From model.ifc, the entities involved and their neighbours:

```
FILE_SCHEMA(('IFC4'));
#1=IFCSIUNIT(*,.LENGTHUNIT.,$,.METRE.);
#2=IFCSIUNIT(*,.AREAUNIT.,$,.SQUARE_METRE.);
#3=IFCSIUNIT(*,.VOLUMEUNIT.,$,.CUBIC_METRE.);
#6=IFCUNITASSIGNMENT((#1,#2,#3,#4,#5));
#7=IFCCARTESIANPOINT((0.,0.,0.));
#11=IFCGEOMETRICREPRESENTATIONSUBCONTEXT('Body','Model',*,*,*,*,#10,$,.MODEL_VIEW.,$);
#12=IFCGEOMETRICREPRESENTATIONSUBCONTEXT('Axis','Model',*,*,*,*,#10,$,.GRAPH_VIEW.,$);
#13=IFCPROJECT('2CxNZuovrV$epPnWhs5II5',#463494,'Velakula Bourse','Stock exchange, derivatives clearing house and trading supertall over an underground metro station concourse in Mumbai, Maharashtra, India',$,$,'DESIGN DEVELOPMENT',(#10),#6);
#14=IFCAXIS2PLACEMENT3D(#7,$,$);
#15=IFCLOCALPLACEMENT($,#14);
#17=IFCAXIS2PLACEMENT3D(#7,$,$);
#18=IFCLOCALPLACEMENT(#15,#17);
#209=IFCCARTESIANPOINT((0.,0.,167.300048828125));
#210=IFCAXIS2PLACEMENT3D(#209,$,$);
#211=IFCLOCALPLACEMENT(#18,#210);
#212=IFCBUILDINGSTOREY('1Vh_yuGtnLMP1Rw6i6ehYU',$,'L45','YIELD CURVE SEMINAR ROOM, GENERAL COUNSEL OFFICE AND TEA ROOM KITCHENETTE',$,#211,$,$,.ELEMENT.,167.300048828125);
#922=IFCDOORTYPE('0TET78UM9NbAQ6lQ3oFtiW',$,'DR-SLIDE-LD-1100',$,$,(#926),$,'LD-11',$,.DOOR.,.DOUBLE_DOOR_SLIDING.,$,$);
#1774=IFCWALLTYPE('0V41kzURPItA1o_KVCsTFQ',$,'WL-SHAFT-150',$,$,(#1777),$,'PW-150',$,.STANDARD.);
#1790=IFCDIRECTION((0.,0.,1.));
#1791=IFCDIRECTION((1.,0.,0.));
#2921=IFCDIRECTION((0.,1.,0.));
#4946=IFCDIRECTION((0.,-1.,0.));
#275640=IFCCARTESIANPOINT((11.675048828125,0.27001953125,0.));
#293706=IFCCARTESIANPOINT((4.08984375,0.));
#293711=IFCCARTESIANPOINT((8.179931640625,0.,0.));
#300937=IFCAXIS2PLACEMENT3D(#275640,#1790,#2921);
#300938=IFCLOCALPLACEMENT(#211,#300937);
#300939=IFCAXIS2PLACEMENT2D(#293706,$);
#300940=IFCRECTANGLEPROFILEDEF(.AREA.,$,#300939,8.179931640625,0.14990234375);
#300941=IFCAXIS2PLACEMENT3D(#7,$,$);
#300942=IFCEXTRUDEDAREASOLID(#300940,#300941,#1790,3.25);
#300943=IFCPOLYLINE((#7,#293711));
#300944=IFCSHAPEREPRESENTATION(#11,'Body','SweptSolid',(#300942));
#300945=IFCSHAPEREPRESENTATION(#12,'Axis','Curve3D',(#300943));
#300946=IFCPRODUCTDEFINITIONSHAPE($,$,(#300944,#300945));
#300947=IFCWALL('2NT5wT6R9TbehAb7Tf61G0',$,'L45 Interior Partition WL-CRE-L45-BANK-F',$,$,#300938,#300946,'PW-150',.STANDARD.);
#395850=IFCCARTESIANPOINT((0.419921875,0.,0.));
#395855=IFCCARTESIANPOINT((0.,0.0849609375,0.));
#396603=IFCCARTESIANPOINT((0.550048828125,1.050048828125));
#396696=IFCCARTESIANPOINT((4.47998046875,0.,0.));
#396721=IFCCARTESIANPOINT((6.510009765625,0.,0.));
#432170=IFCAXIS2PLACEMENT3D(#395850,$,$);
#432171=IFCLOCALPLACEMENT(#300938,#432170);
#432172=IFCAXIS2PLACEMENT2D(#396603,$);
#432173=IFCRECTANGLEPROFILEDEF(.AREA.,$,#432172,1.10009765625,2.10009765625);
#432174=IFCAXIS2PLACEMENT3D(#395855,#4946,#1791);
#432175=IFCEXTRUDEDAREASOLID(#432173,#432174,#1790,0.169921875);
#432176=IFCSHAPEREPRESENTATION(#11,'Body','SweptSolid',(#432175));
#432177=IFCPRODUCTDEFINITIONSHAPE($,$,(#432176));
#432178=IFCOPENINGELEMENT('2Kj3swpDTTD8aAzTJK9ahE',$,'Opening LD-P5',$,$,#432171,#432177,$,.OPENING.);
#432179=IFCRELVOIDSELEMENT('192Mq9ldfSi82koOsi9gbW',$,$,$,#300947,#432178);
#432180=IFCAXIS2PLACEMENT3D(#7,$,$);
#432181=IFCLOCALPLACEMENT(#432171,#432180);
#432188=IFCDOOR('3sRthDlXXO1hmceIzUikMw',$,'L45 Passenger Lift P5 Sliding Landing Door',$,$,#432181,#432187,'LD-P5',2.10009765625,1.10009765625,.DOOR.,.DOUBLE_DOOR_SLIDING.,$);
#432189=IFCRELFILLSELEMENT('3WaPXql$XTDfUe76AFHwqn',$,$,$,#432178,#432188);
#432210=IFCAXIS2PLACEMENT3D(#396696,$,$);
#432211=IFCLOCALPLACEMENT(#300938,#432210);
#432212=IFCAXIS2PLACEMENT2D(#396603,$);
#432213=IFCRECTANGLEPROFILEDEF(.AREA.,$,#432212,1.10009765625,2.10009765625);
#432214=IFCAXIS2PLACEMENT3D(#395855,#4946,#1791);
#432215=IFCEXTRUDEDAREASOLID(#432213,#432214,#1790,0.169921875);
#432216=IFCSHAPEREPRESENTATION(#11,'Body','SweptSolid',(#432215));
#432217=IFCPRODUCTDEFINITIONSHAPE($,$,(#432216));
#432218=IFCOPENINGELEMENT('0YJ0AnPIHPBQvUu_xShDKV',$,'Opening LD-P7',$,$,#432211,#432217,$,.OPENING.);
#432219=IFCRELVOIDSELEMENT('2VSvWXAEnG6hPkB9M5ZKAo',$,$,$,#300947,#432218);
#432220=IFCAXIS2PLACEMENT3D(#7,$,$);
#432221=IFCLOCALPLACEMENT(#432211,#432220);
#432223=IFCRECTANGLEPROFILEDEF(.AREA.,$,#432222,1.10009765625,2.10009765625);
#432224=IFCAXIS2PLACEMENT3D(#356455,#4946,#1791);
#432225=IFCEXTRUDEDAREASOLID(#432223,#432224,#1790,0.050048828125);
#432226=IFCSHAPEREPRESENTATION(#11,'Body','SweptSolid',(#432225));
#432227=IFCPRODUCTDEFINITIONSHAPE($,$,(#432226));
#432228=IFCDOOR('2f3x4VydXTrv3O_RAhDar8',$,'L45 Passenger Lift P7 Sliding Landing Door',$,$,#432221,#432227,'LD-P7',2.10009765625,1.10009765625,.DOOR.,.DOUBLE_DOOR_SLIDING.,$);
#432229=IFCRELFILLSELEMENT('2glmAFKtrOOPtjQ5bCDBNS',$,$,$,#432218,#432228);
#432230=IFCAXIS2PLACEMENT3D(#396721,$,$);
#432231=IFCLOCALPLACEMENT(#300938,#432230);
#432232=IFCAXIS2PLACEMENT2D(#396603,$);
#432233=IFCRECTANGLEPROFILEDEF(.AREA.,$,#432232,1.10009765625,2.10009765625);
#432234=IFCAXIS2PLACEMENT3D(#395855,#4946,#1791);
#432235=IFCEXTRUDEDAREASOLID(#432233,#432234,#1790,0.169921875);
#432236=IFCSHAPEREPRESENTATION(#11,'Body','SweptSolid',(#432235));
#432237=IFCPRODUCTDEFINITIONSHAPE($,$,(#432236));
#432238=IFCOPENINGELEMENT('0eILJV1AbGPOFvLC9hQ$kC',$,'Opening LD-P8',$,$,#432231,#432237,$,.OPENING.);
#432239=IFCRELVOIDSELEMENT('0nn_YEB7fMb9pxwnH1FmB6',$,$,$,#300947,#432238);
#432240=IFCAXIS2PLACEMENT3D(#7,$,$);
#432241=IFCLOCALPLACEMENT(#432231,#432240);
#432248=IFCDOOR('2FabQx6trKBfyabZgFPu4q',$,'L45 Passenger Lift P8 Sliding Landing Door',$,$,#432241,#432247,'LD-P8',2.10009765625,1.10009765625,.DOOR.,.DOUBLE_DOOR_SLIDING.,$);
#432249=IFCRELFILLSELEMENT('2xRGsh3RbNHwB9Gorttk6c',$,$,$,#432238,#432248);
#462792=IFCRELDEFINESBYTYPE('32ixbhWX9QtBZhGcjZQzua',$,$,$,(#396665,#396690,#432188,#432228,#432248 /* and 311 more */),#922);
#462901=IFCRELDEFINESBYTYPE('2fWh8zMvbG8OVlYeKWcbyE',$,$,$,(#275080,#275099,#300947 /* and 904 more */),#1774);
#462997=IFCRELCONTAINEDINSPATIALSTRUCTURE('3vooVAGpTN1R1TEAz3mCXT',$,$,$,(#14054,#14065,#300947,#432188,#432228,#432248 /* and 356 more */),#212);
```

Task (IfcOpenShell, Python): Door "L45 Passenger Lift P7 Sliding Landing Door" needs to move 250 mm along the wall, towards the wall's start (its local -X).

```python
import ifcopenshell
import ifcopenshell.api.geometry
import ifcopenshell.util.placement
import ifcopenshell.util.unit

model = ifcopenshell.open("model.ifc")
unit_scale = ifcopenshell.util.unit.calculate_unit_scale(model)

door = model.by_guid("2f3x4VydXTrv3O_RAhDar8")
opening = door.FillsVoids[0].RelatingOpeningElement
wall = opening.VoidsElements[0].RelatingBuildingElement

wall_matrix = ifcopenshell.util.placement.get_local_placement(wall.ObjectPlacement)
shift = wall_matrix[:3, 0] * -0.25 / unit_scale
before = ifcopenshell.util.placement.get_local_placement(door.ObjectPlacement)[:3, 3].copy()

# The door is placed relative to its opening, so it follows when the opening moves.
matrix = ifcopenshell.util.placement.get_local_placement(opening.ObjectPlacement)
matrix[:3, 3] += shift
ifcopenshell.api.geometry.edit_object_placement(
    model, product=opening, matrix=matrix, is_si=False, should_transform_children=True
)

after = ifcopenshell.util.placement.get_local_placement(door.ObjectPlacement)[:3, 3]
print("door moved by", (after - before).round(3) + 0.0)

model.write("model-out.ifc")
```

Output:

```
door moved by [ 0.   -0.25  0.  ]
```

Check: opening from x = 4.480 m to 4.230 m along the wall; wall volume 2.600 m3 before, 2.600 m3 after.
